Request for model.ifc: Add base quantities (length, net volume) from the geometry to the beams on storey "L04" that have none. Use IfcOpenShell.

First a look at what the model holds.

```python
import ifcopenshell
import ifcopenshell.util.element
import ifcopenshell.util.unit

model = ifcopenshell.open("model.ifc")
print(model.schema)
for unit_type in ("LENGTHUNIT", "AREAUNIT", "VOLUMEUNIT"):
    print(unit_type, ifcopenshell.util.unit.calculate_unit_scale(model, unit_type))
storey = next(s for s in model.by_type("IfcBuildingStorey") if s.Name == "L04")
beams = [e for e in ifcopenshell.util.element.get_decomposition(storey) if e.is_a("IfcBeam")]
for e in sorted(beams, key=lambda e: e.id()):
    print(e.id(), e.is_a(), e.Name, list(ifcopenshell.util.element.get_psets(e, qtos_only=True)), sep=" | ")
```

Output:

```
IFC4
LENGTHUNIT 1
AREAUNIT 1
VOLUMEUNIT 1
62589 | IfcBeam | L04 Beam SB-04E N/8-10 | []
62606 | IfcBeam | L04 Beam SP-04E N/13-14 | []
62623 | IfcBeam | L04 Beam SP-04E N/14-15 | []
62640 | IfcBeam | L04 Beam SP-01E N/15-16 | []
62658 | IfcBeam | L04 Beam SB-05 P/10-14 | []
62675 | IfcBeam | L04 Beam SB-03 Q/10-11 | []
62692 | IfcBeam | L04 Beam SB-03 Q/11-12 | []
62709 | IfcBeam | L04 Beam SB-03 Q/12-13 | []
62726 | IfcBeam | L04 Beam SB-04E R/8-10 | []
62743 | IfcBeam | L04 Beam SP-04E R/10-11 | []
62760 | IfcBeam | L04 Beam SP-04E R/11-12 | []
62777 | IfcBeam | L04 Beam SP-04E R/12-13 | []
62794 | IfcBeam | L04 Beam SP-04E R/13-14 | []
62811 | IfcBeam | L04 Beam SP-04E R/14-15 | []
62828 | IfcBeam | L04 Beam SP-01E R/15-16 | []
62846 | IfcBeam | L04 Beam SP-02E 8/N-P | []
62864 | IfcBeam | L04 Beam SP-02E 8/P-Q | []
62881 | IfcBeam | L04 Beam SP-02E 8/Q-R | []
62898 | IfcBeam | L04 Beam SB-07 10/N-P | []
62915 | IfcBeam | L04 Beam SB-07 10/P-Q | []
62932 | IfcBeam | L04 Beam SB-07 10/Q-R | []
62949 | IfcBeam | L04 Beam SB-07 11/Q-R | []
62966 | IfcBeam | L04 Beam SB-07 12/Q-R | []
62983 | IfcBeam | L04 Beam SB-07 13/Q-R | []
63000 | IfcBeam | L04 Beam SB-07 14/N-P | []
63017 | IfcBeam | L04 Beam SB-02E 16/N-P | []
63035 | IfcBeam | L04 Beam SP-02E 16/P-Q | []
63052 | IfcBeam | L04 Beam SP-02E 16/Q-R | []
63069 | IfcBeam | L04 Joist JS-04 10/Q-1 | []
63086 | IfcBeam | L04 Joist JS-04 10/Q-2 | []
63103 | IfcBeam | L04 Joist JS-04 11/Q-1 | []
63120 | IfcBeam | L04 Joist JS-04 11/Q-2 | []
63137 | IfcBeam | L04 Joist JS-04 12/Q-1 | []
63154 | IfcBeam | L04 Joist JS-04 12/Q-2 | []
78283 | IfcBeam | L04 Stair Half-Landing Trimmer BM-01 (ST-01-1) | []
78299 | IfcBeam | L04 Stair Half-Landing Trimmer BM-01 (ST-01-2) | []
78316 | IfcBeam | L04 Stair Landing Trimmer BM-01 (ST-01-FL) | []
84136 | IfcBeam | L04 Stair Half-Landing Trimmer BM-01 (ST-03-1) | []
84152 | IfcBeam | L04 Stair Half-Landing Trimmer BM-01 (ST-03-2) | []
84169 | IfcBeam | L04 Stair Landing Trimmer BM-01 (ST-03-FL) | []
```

```python
import ifcopenshell
import ifcopenshell.api.pset
import ifcopenshell.geom
import ifcopenshell.util.element
import ifcopenshell.util.shape
import ifcopenshell.util.unit

model = ifcopenshell.open("model.ifc")
unit_scale = ifcopenshell.util.unit.calculate_unit_scale(model)
volume_scale = ifcopenshell.util.unit.calculate_unit_scale(model, "VOLUMEUNIT")
settings = ifcopenshell.geom.settings()

storey = next(s for s in model.by_type("IfcBuildingStorey") if s.Name == "L04")
beams = [e for e in ifcopenshell.util.element.get_decomposition(storey) if e.is_a("IfcBeam")]

for e in sorted(beams, key=lambda e: e.id()):
    if ifcopenshell.util.element.get_psets(e, qtos_only=True, should_inherit=False):
        continue
    # Geometry comes back in metres, in the element's own axes.
    shape = ifcopenshell.geom.create_shape(settings, e)
    values = {
        "Length": ifcopenshell.util.shape.get_max_xyz(shape.geometry) / unit_scale,
        "NetVolume": ifcopenshell.util.shape.get_volume(shape.geometry) / volume_scale,
    }
    qto = ifcopenshell.api.pset.add_qto(model, product=e, name="Qto_BeamBaseQuantities")
    ifcopenshell.api.pset.edit_qto(model, qto=qto, properties=values)
    print(e.id(), {k: round(v, 3) for k, v in values.items()})

model.write("model_edited.ifc")
```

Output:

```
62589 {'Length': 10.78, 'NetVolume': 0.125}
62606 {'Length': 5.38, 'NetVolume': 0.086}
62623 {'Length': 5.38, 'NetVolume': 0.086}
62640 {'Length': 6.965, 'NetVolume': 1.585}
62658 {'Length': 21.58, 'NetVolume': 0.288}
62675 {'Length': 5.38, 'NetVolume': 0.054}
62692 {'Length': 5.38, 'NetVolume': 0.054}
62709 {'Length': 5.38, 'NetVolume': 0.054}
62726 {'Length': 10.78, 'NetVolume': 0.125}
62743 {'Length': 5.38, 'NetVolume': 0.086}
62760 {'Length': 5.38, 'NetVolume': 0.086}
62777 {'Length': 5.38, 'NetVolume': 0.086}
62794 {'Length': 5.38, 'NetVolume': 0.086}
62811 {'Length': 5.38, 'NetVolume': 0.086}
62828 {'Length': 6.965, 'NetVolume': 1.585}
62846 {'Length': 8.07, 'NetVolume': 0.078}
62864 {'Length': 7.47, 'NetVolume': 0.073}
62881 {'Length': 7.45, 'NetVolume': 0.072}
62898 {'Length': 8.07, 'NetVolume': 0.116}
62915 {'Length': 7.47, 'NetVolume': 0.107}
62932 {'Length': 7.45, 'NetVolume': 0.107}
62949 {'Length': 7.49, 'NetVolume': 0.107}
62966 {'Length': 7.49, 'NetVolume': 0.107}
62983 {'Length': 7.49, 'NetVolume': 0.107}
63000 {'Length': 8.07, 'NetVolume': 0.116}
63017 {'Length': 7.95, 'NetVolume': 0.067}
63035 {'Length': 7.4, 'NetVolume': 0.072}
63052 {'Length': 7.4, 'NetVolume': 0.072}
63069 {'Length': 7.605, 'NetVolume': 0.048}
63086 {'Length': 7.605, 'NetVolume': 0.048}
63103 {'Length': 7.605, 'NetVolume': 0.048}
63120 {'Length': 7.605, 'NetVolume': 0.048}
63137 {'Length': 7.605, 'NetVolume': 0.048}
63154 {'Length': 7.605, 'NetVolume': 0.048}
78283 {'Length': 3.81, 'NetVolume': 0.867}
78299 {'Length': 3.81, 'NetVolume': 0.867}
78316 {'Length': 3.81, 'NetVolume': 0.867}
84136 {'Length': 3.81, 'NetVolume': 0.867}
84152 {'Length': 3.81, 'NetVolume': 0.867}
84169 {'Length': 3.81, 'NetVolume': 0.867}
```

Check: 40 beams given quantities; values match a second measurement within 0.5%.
